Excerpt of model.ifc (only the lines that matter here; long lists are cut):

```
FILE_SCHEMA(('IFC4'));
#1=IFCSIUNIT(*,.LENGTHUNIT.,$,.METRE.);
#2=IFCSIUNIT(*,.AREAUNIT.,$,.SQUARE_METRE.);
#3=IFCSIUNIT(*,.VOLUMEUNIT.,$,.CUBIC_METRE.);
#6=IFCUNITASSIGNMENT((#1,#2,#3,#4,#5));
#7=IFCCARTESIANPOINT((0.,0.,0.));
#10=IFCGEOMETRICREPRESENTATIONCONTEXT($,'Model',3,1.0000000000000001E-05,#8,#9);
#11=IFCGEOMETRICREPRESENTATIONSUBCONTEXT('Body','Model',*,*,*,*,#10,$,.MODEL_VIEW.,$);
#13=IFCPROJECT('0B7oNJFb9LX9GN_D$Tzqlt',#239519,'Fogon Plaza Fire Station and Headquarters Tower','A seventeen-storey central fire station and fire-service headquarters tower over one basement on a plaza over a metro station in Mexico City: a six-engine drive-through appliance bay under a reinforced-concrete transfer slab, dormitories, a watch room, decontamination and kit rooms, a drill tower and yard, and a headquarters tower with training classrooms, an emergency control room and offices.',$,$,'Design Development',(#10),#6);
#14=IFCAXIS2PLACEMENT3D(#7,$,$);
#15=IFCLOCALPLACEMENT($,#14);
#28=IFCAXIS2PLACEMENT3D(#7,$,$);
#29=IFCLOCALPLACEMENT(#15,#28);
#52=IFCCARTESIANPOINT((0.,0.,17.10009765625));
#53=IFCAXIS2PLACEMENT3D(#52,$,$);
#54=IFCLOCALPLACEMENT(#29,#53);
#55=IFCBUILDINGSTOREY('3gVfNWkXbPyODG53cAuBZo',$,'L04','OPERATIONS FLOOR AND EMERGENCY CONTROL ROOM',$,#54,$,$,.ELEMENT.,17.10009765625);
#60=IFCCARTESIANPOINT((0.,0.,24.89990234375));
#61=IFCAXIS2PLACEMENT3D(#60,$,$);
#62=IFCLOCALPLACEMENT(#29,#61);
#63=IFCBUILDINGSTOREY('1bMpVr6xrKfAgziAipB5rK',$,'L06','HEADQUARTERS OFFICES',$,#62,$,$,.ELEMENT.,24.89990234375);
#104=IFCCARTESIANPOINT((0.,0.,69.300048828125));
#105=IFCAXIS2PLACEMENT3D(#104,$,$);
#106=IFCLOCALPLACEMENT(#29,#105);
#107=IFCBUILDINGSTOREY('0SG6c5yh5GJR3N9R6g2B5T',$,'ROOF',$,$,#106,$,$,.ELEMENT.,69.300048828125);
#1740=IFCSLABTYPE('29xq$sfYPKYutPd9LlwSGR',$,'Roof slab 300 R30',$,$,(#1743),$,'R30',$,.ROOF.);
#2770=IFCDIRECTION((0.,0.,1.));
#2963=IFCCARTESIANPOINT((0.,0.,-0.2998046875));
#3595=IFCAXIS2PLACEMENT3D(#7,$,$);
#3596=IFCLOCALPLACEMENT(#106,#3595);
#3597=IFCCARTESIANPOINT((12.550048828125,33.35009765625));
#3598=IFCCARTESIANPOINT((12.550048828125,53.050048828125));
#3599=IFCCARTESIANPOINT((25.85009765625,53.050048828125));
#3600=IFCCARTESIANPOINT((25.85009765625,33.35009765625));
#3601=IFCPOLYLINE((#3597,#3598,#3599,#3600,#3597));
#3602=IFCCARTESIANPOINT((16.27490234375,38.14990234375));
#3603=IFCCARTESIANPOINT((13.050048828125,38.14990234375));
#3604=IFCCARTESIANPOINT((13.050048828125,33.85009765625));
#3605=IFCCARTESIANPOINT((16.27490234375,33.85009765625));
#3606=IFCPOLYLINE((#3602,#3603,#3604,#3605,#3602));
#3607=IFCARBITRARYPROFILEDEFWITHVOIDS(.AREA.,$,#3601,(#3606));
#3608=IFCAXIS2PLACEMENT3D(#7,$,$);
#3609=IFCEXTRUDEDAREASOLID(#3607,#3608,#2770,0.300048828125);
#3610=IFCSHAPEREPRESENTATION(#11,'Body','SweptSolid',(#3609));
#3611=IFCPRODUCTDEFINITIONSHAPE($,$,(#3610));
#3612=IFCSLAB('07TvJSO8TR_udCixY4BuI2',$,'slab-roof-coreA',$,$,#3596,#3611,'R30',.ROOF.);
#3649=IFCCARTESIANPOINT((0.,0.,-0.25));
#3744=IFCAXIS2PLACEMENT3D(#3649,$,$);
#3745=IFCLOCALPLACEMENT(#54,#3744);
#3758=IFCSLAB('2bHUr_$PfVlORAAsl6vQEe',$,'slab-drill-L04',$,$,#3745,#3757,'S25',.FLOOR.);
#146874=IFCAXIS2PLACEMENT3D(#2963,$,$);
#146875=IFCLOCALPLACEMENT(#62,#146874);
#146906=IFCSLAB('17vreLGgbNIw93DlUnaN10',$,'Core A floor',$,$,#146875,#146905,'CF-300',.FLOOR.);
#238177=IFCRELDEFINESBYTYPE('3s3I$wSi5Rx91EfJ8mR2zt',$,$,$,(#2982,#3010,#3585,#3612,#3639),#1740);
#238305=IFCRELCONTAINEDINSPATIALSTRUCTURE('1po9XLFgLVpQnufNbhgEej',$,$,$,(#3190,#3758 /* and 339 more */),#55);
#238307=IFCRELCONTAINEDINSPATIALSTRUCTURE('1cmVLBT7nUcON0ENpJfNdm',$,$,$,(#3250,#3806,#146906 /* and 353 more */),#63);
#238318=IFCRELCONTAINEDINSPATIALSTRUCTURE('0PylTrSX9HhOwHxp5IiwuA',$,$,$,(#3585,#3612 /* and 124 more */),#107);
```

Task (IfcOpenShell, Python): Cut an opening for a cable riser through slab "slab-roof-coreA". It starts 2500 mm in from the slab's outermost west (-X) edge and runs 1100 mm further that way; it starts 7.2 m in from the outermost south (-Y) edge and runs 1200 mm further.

```python
import numpy as np
import ifcopenshell
import ifcopenshell.api.feature
import ifcopenshell.api.geometry
import ifcopenshell.api.root
import ifcopenshell.geom
import ifcopenshell.util.placement
import ifcopenshell.util.representation
import ifcopenshell.util.shape
import ifcopenshell.util.unit

model = ifcopenshell.open("model.ifc")
unit_scale = ifcopenshell.util.unit.calculate_unit_scale(model)
settings = ifcopenshell.geom.settings()


def volume(element):
    """Net volume in cubic metres, openings subtracted."""
    shape = ifcopenshell.geom.create_shape(settings, element)
    return ifcopenshell.util.shape.get_volume(shape.geometry)


slab = model.by_id(3612)
before = volume(slab)

# Extent in the slab's own axes, in metres. The edges named are its -X and -Y sides.
slab_shape = ifcopenshell.geom.create_shape(settings, slab)
vertices = ifcopenshell.util.shape.get_vertices(slab_shape.geometry)
x_min, y_min, bottom = vertices.min(axis=0)
top = vertices[:, 2].max()

opening = ifcopenshell.api.root.create_entity(model, ifc_class="IfcOpeningElement", name="Cable riser opening", predefined_type="OPENING")
context = ifcopenshell.util.representation.get_context(model, "Model", "Body", "MODEL_VIEW")
width, depth = 1.1, 1.2
outline = [(0.0, 0.0), (width, 0.0), (width, depth), (0.0, depth), (0.0, 0.0)]
# Overshoot both faces by 50 mm so the cut is clean.
shape = ifcopenshell.api.geometry.add_slab_representation(
    model, context=context, depth=top - bottom + 0.1, polyline=outline
)
ifcopenshell.api.geometry.assign_representation(model, product=opening, representation=shape)

matrix = ifcopenshell.util.placement.get_local_placement(slab.ObjectPlacement)
matrix[:, 3] = matrix @ np.append(np.array([x_min + 2.5, y_min + 7.2, bottom - 0.05]) / unit_scale, 1.0)
ifcopenshell.api.geometry.edit_object_placement(model, product=opening, matrix=matrix, is_si=False)
ifcopenshell.api.feature.add_feature(model, feature=opening, element=slab)

after = volume(slab)

print(f"slab volume {before:.3f} -> {after:.3f} m3")

model.write("model_edited.ifc")
```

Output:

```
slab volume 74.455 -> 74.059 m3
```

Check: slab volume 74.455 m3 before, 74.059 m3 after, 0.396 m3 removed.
